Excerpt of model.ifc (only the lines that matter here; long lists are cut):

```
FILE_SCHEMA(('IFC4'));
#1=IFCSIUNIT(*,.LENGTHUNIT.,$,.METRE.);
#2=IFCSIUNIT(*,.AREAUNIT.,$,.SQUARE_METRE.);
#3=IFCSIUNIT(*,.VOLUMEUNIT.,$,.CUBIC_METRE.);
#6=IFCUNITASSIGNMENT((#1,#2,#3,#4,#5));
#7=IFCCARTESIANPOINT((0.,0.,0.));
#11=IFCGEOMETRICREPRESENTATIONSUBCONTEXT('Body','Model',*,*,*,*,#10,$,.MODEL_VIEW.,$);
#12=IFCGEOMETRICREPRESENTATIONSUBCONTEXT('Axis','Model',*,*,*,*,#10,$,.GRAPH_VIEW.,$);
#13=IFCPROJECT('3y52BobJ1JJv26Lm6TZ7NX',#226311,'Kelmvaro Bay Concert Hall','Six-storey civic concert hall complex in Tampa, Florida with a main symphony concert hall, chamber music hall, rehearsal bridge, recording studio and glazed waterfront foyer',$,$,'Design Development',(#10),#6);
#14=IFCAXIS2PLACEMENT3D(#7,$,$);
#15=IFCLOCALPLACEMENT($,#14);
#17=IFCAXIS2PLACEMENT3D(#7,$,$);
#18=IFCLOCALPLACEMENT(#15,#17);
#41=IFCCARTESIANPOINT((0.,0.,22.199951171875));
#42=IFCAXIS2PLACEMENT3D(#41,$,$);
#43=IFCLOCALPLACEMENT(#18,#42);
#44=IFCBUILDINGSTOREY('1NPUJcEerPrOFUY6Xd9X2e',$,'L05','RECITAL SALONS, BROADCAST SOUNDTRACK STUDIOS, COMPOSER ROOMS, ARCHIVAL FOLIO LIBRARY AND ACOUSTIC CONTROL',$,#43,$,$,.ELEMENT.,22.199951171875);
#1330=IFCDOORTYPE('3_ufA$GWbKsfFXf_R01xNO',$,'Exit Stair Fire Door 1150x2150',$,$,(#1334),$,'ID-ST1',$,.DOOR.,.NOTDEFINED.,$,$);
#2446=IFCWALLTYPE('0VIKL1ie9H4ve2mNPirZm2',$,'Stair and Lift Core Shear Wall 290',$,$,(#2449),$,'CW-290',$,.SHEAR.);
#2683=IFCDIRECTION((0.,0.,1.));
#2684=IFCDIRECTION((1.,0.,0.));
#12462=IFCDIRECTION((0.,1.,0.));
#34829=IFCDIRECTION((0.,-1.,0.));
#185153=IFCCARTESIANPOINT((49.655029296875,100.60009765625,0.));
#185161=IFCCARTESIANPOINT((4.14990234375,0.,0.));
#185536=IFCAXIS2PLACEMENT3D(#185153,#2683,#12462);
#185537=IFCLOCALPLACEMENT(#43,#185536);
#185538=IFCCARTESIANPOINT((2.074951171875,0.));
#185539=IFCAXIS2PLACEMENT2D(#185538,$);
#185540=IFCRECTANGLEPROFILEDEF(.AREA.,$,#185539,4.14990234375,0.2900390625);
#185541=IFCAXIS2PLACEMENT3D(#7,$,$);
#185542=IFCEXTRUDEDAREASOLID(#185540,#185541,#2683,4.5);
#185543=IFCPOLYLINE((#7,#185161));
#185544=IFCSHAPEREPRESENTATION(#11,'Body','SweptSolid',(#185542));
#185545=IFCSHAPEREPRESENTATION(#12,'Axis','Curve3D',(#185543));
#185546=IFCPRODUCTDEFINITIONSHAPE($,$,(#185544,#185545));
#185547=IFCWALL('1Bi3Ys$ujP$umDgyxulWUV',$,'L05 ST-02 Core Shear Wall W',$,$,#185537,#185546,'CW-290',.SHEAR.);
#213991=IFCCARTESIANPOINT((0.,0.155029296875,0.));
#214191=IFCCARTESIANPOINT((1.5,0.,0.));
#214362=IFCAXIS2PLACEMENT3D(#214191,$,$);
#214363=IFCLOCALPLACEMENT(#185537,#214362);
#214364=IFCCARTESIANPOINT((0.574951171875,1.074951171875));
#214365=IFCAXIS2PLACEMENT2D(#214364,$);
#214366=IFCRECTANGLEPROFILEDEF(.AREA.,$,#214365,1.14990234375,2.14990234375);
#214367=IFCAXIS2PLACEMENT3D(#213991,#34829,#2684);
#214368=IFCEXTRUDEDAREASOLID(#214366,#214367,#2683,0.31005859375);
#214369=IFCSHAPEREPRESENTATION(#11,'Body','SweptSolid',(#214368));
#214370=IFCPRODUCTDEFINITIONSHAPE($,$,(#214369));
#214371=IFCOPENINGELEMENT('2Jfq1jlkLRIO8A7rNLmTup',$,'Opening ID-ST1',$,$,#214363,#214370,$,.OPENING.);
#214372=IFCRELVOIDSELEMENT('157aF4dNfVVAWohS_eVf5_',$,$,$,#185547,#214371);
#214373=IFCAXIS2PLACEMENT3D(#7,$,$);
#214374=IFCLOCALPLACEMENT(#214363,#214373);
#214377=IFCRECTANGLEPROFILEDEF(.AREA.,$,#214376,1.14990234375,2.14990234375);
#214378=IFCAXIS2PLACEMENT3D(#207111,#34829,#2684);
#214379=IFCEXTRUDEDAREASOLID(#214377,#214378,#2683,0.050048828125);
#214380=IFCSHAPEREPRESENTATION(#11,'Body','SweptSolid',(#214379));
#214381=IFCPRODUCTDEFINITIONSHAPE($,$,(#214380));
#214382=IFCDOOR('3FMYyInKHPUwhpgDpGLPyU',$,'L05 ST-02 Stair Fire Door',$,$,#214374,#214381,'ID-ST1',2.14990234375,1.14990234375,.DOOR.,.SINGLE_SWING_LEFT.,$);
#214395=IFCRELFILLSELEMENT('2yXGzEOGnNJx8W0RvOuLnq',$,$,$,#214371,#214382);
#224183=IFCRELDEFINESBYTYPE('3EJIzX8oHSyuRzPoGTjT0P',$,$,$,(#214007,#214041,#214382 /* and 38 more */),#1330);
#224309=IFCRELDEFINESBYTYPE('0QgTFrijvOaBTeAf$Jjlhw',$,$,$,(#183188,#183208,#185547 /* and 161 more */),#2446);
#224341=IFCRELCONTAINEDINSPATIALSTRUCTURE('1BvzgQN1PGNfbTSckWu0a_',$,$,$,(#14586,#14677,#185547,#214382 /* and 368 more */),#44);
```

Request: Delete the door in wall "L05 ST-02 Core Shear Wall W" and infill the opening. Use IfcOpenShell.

```python
import ifcopenshell
import ifcopenshell.api.feature
import ifcopenshell.api.root
import ifcopenshell.geom
import ifcopenshell.util.shape

model = ifcopenshell.open("model.ifc")
settings = ifcopenshell.geom.settings()


def volume(element):
    """Net volume in cubic metres, openings subtracted."""
    shape = ifcopenshell.geom.create_shape(settings, element)
    return ifcopenshell.util.shape.get_volume(shape.geometry)


door = model.by_guid("3FMYyInKHPUwhpgDpGLPyU")
opening = door.FillsVoids[0].RelatingOpeningElement
wall = opening.VoidsElements[0].RelatingBuildingElement
before = volume(wall)

ifcopenshell.api.root.remove_product(model, product=door)
ifcopenshell.api.feature.remove_feature(model, feature=opening)

after = volume(wall)

print(f"wall volume {before:.3f} -> {after:.3f} m3")

model.write("model_edited.ifc")
```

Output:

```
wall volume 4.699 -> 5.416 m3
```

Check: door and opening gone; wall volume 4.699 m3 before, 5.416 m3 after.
